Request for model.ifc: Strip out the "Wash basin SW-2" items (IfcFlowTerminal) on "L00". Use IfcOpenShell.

First a look at what the model holds.

```python
import ifcopenshell
import ifcopenshell.util.element

model = ifcopenshell.open("model.ifc")
print(model.schema)
storey = next(s for s in model.by_type("IfcBuildingStorey") if s.Name == "L00")
terminals = [e for e in ifcopenshell.util.element.get_decomposition(storey) if e.is_a("IfcFlowTerminal")]
seen = {}
for e in terminals:
    element_type = ifcopenshell.util.element.get_type(e)
    name = element_type.Name if element_type not in (None, e) else None
    seen[name] = seen.get(name, 0) + 1
for name, count in sorted(seen.items(), key=str):
    print(count, "x", name)
```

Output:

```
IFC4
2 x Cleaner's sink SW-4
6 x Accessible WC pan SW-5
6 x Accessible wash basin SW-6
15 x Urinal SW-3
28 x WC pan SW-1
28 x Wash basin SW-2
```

```python
import ifcopenshell
import ifcopenshell.api.root
import ifcopenshell.util.element

model = ifcopenshell.open("model.ifc")

storey = next(s for s in model.by_type("IfcBuildingStorey") if s.Name == "L00")
terminals = [e for e in ifcopenshell.util.element.get_decomposition(storey) if e.is_a("IfcFlowTerminal")]
targets = [e for e in terminals if (t := ifcopenshell.util.element.get_type(e)) not in (None, e) and t.Name == "Wash basin SW-2"]

for e in targets:
    ifcopenshell.api.root.remove_product(model, product=e)
print(len(targets), "removed")

model.write("model-out.ifc")
```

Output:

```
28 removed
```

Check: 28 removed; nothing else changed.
